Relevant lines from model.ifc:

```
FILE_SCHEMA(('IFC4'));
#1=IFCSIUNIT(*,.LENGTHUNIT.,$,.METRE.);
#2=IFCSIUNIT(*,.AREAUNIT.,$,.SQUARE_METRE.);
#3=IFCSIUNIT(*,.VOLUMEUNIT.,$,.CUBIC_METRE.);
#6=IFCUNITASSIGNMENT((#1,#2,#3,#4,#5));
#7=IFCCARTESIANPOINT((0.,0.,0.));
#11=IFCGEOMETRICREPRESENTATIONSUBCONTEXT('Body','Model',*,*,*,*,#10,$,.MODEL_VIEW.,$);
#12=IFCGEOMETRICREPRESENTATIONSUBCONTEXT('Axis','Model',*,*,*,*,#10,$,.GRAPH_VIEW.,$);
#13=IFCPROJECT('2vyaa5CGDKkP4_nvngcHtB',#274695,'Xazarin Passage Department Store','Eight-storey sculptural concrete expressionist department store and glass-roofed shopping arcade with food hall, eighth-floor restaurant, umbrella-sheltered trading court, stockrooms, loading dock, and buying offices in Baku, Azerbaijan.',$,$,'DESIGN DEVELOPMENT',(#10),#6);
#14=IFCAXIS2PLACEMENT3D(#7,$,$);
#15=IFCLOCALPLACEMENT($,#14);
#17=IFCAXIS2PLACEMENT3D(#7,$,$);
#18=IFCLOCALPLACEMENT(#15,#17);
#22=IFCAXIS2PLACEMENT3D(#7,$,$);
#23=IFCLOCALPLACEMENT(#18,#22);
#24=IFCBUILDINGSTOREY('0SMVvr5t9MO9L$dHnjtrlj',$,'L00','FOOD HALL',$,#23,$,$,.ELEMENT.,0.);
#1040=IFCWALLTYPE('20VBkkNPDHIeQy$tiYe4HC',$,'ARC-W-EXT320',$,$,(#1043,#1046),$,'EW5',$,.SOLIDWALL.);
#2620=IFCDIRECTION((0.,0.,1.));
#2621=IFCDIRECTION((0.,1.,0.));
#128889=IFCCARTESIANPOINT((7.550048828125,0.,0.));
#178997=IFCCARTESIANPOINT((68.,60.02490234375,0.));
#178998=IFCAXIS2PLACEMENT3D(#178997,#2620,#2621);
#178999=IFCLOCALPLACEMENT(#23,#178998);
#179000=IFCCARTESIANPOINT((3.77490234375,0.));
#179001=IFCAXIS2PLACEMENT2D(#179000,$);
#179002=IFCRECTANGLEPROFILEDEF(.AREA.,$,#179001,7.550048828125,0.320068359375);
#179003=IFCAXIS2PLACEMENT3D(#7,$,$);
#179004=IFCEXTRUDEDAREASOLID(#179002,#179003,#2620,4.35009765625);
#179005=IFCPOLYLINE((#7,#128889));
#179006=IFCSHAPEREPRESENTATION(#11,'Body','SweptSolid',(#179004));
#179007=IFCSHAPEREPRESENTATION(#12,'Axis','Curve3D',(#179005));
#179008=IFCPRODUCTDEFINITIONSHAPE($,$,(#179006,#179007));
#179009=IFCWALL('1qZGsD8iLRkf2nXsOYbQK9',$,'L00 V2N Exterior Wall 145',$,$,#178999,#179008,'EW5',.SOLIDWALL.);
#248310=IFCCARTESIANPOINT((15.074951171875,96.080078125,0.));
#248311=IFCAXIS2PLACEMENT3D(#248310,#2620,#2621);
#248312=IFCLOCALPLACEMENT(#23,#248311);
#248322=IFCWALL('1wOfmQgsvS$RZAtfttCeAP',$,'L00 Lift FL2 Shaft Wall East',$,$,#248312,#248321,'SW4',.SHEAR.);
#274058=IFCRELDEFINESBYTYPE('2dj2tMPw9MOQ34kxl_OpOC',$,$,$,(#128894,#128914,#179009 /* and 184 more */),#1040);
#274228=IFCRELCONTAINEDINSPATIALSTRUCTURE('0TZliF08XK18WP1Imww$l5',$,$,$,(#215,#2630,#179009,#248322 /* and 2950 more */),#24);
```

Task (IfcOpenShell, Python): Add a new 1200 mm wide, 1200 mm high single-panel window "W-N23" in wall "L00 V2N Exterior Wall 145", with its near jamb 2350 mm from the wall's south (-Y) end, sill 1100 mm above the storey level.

```python
import numpy as np
import ifcopenshell
import ifcopenshell.api.feature
import ifcopenshell.api.geometry
import ifcopenshell.api.root
import ifcopenshell.api.spatial
import ifcopenshell.geom
import ifcopenshell.util.element
import ifcopenshell.util.placement
import ifcopenshell.util.representation
import ifcopenshell.util.shape
import ifcopenshell.util.unit

model = ifcopenshell.open("model.ifc")
unit_scale = ifcopenshell.util.unit.calculate_unit_scale(model)
settings = ifcopenshell.geom.settings()


def volume(element):
    """Net volume in cubic metres, openings subtracted."""
    shape = ifcopenshell.geom.create_shape(settings, element)
    return ifcopenshell.util.shape.get_volume(shape.geometry)


wall = model.by_guid("1qZGsD8iLRkf2nXsOYbQK9")
storey = ifcopenshell.util.element.get_container(wall, ifc_class="IfcBuildingStorey")
context = ifcopenshell.util.representation.get_context(model, "Model", "Body", "MODEL_VIEW")
before = volume(wall)

width, height, from_end, sill = 1.2, 1.2, 2.35, 1.1  # metres

# The wall runs along its own X axis, and the end named is its -X end.
wall_shape = ifcopenshell.geom.create_shape(settings, wall)
x, y, z = ifcopenshell.util.shape.get_vertices(wall_shape.geometry).T
start = x.min() + from_end
face, thickness = float(y.min()), float(y.max() - y.min())
wall_matrix = ifcopenshell.util.placement.get_local_placement(wall.ObjectPlacement)
level = ifcopenshell.util.placement.get_local_placement(storey.ObjectPlacement)[2, 3]


def in_wall(x, y):
    """Placement at x, y metres in the wall's axes, at sill height."""
    matrix = wall_matrix.copy()
    matrix[:, 3] = wall_matrix @ np.array([x / unit_scale, y / unit_scale, 0.0, 1.0])
    matrix[2, 3] = level + sill / unit_scale
    return matrix


# Opening: a box that overshoots both wall faces by 50 mm.
opening = ifcopenshell.api.root.create_entity(model, ifc_class="IfcOpeningElement", predefined_type="OPENING")
box = ifcopenshell.api.geometry.add_wall_representation(
    model, context=context, length=width, height=height, thickness=thickness + 0.1
)
ifcopenshell.api.geometry.assign_representation(model, product=opening, representation=box)
ifcopenshell.api.geometry.edit_object_placement(model, product=opening, matrix=in_wall(start, face - 0.05), is_si=False)
ifcopenshell.api.feature.add_feature(model, feature=opening, element=wall)

window = ifcopenshell.api.root.create_entity(model, ifc_class="IfcWindow", name="W-N23", predefined_type="WINDOW")
window.OverallWidth, window.OverallHeight = width / unit_scale, height / unit_scale
window.PartitioningType = "SINGLE_PANEL"
body = ifcopenshell.api.geometry.add_window_representation(
    model,
    context=context,
    overall_width=window.OverallWidth,
    overall_height=window.OverallHeight,
    partition_type="SINGLE_PANEL",
)
ifcopenshell.api.geometry.assign_representation(model, product=window, representation=body)
ifcopenshell.api.spatial.assign_container(model, products=[window], relating_structure=storey)
ifcopenshell.api.feature.add_filling(model, opening=opening, element=window)

# Centre the window in the wall's thickness.
ifcopenshell.api.geometry.edit_object_placement(model, product=window, matrix=in_wall(start, face), is_si=False)
window_shape = ifcopenshell.geom.create_shape(settings, window)
depth = ifcopenshell.util.shape.get_vertices(window_shape.geometry)[:, 1]
offset = face + thickness / 2 - (depth.min() + depth.max()) / 2
ifcopenshell.api.geometry.edit_object_placement(model, product=window, matrix=in_wall(start, offset), is_si=False)

after = volume(wall)

print(f"wall volume {before:.3f} -> {after:.3f} m3")

model.write("model-out.ifc")
```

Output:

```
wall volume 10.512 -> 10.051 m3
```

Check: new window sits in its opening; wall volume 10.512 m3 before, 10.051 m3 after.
